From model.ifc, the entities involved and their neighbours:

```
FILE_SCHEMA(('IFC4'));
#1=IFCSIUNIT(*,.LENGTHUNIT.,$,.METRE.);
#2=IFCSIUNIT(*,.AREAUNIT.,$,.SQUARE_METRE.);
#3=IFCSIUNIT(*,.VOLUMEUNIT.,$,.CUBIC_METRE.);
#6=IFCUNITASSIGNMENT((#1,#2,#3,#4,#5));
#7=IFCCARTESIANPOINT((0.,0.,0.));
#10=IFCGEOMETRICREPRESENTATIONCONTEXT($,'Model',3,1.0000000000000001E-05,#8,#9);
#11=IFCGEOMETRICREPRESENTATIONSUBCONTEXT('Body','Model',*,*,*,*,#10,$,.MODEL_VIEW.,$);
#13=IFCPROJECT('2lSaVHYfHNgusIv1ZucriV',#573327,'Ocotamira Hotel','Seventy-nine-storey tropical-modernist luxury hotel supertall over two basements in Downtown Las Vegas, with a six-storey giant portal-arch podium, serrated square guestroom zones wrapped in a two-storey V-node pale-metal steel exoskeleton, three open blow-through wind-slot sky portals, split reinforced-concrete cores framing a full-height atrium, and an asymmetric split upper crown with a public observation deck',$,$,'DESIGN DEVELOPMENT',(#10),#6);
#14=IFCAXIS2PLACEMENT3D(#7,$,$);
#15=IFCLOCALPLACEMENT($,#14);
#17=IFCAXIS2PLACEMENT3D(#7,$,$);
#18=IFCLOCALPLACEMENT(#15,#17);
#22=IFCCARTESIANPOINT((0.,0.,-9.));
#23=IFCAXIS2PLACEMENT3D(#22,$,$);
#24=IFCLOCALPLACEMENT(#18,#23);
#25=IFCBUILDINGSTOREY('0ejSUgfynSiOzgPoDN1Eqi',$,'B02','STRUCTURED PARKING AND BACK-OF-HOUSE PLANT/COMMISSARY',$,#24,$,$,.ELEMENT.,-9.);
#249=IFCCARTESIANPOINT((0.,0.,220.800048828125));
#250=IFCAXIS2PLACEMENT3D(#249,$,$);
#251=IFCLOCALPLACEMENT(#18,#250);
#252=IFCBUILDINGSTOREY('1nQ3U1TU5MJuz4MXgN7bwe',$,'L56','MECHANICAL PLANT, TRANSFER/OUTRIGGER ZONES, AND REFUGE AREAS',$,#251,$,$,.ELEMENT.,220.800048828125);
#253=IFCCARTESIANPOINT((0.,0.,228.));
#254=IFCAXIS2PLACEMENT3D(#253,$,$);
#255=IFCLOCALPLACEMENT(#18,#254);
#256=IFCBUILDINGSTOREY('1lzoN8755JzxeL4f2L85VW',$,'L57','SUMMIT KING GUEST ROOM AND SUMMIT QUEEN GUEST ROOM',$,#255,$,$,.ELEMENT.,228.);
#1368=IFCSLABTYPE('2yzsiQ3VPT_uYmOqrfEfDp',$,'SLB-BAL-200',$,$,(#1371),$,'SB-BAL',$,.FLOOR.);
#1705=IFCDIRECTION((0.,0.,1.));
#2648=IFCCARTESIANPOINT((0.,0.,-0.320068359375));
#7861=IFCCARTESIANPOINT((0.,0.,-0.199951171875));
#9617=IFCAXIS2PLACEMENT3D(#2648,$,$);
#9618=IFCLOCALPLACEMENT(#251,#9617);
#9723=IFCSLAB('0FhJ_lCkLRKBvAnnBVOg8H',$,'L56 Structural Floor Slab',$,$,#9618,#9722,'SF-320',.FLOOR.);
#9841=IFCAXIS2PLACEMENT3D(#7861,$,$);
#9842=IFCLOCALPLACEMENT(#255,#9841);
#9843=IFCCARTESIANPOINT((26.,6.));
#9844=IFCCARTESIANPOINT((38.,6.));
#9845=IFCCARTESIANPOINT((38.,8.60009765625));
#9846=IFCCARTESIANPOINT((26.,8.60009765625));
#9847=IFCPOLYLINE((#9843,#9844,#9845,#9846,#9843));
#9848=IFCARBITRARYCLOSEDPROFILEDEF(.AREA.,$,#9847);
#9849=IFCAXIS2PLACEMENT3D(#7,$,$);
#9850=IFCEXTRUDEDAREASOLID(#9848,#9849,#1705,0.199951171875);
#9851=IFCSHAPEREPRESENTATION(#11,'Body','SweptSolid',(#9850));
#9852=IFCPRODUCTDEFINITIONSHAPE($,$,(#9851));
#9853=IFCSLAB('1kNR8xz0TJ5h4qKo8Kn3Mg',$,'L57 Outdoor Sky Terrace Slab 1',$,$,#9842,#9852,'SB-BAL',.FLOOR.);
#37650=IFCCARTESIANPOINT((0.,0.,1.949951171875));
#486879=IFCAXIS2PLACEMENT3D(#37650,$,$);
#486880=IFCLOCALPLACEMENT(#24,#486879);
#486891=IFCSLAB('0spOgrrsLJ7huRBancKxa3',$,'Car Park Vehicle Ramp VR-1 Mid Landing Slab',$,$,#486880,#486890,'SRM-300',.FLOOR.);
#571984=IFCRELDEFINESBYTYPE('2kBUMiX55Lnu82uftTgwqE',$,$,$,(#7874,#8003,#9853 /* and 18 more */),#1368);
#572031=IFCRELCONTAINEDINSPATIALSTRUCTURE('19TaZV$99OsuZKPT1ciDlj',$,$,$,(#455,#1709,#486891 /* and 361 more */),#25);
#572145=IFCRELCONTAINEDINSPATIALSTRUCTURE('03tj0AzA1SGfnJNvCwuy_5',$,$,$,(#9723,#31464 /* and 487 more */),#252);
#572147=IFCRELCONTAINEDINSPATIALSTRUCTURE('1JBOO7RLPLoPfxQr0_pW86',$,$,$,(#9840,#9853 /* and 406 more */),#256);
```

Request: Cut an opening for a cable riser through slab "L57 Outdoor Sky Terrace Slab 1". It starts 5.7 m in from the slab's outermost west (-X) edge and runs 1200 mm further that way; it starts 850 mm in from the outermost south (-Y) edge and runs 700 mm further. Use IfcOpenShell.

```python
import numpy as np
import ifcopenshell
import ifcopenshell.api.feature
import ifcopenshell.api.geometry
import ifcopenshell.api.root
import ifcopenshell.geom
import ifcopenshell.util.placement
import ifcopenshell.util.representation
import ifcopenshell.util.shape
import ifcopenshell.util.unit

model = ifcopenshell.open("model.ifc")
unit_scale = ifcopenshell.util.unit.calculate_unit_scale(model)
settings = ifcopenshell.geom.settings()


def volume(element):
    """Net volume in cubic metres, openings subtracted."""
    shape = ifcopenshell.geom.create_shape(settings, element)
    return ifcopenshell.util.shape.get_volume(shape.geometry)


slab = model.by_id(9853)
before = volume(slab)

# Extent in the slab's own axes, in metres. The edges named are its -X and -Y sides.
slab_shape = ifcopenshell.geom.create_shape(settings, slab)
vertices = ifcopenshell.util.shape.get_vertices(slab_shape.geometry)
x_min, y_min, bottom = vertices.min(axis=0)
top = vertices[:, 2].max()

opening = ifcopenshell.api.root.create_entity(model, ifc_class="IfcOpeningElement", name="Cable riser opening", predefined_type="OPENING")
context = ifcopenshell.util.representation.get_context(model, "Model", "Body", "MODEL_VIEW")
width, depth = 1.2, 0.7
outline = [(0.0, 0.0), (width, 0.0), (width, depth), (0.0, depth), (0.0, 0.0)]
# Overshoot both faces by 50 mm so the cut is clean.
shape = ifcopenshell.api.geometry.add_slab_representation(
    model, context=context, depth=top - bottom + 0.1, polyline=outline
)
ifcopenshell.api.geometry.assign_representation(model, product=opening, representation=shape)

matrix = ifcopenshell.util.placement.get_local_placement(slab.ObjectPlacement)
matrix[:, 3] = matrix @ np.append(np.array([x_min + 5.7, y_min + 0.85, bottom - 0.05]) / unit_scale, 1.0)
ifcopenshell.api.geometry.edit_object_placement(model, product=opening, matrix=matrix, is_si=False)
ifcopenshell.api.feature.add_feature(model, feature=opening, element=slab)

after = volume(slab)

print(f"slab volume {before:.3f} -> {after:.3f} m3")

model.write("model-out.ifc")
```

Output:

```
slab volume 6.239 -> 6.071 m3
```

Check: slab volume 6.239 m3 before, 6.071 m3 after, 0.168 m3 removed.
